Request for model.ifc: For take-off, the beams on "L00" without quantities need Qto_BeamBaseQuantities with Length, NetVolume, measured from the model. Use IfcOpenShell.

First a look at what the model holds.

```python
import ifcopenshell
import ifcopenshell.util.element
import ifcopenshell.util.unit

model = ifcopenshell.open("model.ifc")
print(model.schema)
for unit_type in ("LENGTHUNIT", "AREAUNIT", "VOLUMEUNIT"):
    print(unit_type, ifcopenshell.util.unit.calculate_unit_scale(model, unit_type))
storey = next(s for s in model.by_type("IfcBuildingStorey") if s.Name == "L00")
beams = [e for e in ifcopenshell.util.element.get_decomposition(storey) if e.is_a("IfcBeam")]
for e in sorted(beams, key=lambda e: e.id()):
    print(e.id(), e.is_a(), e.Name, list(ifcopenshell.util.element.get_psets(e, qtos_only=True)), sep=" | ")
```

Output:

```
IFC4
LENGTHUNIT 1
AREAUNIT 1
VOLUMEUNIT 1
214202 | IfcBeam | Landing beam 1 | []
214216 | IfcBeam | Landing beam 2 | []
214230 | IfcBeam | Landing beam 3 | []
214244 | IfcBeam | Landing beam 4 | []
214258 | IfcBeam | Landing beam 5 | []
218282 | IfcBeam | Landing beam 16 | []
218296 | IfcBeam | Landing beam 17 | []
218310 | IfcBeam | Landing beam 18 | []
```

```python
import ifcopenshell
import ifcopenshell.api.pset
import ifcopenshell.geom
import ifcopenshell.util.element
import ifcopenshell.util.shape
import ifcopenshell.util.unit

model = ifcopenshell.open("model.ifc")
unit_scale = ifcopenshell.util.unit.calculate_unit_scale(model)
volume_scale = ifcopenshell.util.unit.calculate_unit_scale(model, "VOLUMEUNIT")
settings = ifcopenshell.geom.settings()

storey = next(s for s in model.by_type("IfcBuildingStorey") if s.Name == "L00")
beams = [e for e in ifcopenshell.util.element.get_decomposition(storey) if e.is_a("IfcBeam")]

for e in sorted(beams, key=lambda e: e.id()):
    if ifcopenshell.util.element.get_psets(e, qtos_only=True, should_inherit=False):
        continue
    # Geometry comes back in metres, in the element's own axes.
    shape = ifcopenshell.geom.create_shape(settings, e)
    values = {
        "Length": ifcopenshell.util.shape.get_max_xyz(shape.geometry) / unit_scale,
        "NetVolume": ifcopenshell.util.shape.get_volume(shape.geometry) / volume_scale,
    }
    qto = ifcopenshell.api.pset.add_qto(model, product=e, name="Qto_BeamBaseQuantities")
    ifcopenshell.api.pset.edit_qto(model, qto=qto, properties=values)
    print(e.id(), {k: round(v, 3) for k, v in values.items()})

model.write("model-out.ifc")
```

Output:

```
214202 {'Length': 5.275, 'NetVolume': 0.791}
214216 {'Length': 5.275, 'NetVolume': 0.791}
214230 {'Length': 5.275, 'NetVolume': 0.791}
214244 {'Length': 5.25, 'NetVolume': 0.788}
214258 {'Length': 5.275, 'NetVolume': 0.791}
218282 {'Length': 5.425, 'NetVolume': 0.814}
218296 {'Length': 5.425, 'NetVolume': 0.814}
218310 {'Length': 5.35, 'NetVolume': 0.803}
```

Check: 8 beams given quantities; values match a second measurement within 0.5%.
